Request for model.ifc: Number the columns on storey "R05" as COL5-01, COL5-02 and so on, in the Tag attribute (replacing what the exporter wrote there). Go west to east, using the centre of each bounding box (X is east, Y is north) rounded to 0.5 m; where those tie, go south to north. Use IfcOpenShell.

First a look at what the model holds.

```python
import ifcopenshell
import ifcopenshell.util.element
import ifcopenshell.util.placement

model = ifcopenshell.open("model.ifc")
print(model.schema)
storey = next(s for s in model.by_type("IfcBuildingStorey") if s.Name == "R05")
columns = [e for e in ifcopenshell.util.element.get_decomposition(storey) if e.is_a("IfcColumn")]
for e in sorted(columns, key=lambda e: e.id()):
    origin = ifcopenshell.util.placement.get_local_placement(e.ObjectPlacement)[:3, 3]
    print(e.id(), e.Tag, e.Name, origin.round(2) + 0.0, sep=" | ")
```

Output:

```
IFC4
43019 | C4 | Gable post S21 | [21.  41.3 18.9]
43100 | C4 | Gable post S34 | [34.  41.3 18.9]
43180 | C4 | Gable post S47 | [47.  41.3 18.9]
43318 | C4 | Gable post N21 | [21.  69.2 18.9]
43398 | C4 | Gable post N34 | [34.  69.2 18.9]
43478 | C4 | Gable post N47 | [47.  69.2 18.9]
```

```python
import ifcopenshell
import ifcopenshell.geom
import ifcopenshell.util.element
import ifcopenshell.util.shape

model = ifcopenshell.open("model.ifc")
settings = ifcopenshell.geom.settings()
settings.set("use-world-coords", True)


def centre(element):
    shape = ifcopenshell.geom.create_shape(settings, element)
    return ifcopenshell.util.shape.get_bbox_centroid(shape.geometry)


storey = next(s for s in model.by_type("IfcBuildingStorey") if s.Name == "R05")
columns = [e for e in ifcopenshell.util.element.get_decomposition(storey) if e.is_a("IfcColumn")]

# Insertion points can sit at a corner or the storey origin, so sort by the geometry (in metres).
centres = {e: centre(e) for e in columns}
columns.sort(key=lambda e: (round(centres[e][0] / 0.5), centres[e][1]))

for i, e in enumerate(columns, start=1):
    number = f"COL5-{i:02d}"
    e.Tag = number
    print(e.id(), number)

model.write("model_v2.ifc")
```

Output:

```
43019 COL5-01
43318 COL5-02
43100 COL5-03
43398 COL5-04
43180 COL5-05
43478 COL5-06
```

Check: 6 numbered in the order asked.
